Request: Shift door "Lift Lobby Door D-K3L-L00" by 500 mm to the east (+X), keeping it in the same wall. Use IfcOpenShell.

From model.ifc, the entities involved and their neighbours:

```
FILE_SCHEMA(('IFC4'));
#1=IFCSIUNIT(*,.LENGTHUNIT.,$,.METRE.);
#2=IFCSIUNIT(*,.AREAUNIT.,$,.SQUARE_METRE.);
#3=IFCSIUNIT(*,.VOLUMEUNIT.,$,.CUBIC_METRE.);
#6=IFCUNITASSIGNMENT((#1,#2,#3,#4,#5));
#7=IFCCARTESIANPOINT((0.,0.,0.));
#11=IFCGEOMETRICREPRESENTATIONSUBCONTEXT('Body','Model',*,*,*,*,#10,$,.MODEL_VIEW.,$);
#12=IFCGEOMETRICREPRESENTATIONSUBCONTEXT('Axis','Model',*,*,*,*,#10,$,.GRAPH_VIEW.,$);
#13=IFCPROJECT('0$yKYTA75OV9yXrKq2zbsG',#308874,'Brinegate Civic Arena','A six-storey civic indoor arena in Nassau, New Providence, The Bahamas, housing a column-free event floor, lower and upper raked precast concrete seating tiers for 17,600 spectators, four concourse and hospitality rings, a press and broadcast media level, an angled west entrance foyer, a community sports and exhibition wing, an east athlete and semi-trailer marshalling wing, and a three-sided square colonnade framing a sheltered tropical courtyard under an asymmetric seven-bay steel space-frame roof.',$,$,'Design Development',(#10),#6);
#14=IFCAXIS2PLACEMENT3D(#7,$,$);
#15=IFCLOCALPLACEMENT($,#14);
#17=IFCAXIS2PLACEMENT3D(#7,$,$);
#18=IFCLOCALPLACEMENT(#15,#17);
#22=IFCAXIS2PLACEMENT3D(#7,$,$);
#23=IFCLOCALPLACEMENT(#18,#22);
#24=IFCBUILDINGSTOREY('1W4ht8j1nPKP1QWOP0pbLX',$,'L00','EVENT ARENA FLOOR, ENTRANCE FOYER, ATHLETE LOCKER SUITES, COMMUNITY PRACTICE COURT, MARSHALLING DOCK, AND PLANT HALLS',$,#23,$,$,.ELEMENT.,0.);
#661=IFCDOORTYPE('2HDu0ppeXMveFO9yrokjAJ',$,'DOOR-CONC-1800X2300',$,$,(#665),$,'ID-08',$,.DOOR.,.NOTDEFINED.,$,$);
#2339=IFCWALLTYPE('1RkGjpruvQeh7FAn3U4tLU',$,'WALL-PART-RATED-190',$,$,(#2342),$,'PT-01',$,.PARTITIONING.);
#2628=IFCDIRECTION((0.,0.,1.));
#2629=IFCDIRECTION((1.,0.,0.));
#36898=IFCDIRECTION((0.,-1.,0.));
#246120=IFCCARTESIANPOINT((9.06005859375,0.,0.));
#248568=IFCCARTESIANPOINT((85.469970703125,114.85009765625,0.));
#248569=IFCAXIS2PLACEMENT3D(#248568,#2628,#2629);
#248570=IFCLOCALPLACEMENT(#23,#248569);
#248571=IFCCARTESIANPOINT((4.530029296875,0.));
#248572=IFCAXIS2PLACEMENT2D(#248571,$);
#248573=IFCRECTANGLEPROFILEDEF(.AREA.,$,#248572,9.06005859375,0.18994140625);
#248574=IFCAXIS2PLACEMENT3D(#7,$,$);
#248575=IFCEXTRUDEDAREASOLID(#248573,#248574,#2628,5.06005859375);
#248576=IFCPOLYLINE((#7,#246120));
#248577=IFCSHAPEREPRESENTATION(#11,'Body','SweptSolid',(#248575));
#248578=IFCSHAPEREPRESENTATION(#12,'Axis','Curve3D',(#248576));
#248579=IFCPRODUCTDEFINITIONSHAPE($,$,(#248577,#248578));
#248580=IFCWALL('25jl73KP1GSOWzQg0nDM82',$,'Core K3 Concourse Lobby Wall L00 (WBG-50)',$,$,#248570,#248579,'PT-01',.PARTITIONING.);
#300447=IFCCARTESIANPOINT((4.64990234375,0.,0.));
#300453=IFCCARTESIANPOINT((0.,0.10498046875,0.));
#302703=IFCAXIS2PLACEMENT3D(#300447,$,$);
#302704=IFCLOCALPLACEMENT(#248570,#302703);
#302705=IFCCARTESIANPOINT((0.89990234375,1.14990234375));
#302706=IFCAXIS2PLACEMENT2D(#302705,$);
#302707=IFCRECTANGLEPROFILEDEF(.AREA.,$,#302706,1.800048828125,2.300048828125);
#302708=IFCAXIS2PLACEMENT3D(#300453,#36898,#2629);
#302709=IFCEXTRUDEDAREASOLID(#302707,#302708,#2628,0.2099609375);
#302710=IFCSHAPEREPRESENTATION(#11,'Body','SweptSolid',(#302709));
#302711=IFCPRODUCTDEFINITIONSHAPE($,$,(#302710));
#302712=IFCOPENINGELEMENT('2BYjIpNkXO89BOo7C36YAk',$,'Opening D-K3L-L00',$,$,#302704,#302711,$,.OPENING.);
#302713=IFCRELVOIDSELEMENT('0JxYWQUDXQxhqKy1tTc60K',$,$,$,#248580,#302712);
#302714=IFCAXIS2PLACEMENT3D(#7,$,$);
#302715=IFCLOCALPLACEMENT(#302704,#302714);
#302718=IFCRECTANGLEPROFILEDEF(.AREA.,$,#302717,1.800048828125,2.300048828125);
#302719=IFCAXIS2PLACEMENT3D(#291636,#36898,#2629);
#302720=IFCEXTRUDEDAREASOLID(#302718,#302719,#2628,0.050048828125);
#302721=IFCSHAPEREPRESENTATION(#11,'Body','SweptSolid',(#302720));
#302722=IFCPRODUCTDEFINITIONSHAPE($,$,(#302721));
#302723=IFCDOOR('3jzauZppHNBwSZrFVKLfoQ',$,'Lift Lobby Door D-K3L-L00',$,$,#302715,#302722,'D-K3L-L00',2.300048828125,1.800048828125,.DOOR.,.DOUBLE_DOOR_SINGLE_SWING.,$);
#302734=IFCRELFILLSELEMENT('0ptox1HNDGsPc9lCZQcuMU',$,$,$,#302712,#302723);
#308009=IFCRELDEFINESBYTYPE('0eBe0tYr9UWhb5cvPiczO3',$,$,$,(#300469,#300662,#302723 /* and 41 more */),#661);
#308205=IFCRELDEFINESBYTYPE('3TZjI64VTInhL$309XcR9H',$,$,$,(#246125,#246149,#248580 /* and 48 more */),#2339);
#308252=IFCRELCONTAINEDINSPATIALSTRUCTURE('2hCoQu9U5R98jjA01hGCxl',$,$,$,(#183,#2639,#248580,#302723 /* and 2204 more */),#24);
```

```python
import ifcopenshell
import ifcopenshell.api.geometry
import ifcopenshell.util.placement
import ifcopenshell.util.unit

model = ifcopenshell.open("model.ifc")
unit_scale = ifcopenshell.util.unit.calculate_unit_scale(model)

door = model.by_id(302723)
opening = door.FillsVoids[0].RelatingOpeningElement
wall = opening.VoidsElements[0].RelatingBuildingElement

wall_matrix = ifcopenshell.util.placement.get_local_placement(wall.ObjectPlacement)
shift = wall_matrix[:3, 0] * 0.5 / unit_scale
before = ifcopenshell.util.placement.get_local_placement(door.ObjectPlacement)[:3, 3].copy()

# The door is placed relative to its opening, so it follows when the opening moves.
matrix = ifcopenshell.util.placement.get_local_placement(opening.ObjectPlacement)
matrix[:3, 3] += shift
ifcopenshell.api.geometry.edit_object_placement(
    model, product=opening, matrix=matrix, is_si=False, should_transform_children=True
)

after = ifcopenshell.util.placement.get_local_placement(door.ObjectPlacement)[:3, 3]
print("door moved by", (after - before).round(3) + 0.0)

model.write("model_rev.ifc")
```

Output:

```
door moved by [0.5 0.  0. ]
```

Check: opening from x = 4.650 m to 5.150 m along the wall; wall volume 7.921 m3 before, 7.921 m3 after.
